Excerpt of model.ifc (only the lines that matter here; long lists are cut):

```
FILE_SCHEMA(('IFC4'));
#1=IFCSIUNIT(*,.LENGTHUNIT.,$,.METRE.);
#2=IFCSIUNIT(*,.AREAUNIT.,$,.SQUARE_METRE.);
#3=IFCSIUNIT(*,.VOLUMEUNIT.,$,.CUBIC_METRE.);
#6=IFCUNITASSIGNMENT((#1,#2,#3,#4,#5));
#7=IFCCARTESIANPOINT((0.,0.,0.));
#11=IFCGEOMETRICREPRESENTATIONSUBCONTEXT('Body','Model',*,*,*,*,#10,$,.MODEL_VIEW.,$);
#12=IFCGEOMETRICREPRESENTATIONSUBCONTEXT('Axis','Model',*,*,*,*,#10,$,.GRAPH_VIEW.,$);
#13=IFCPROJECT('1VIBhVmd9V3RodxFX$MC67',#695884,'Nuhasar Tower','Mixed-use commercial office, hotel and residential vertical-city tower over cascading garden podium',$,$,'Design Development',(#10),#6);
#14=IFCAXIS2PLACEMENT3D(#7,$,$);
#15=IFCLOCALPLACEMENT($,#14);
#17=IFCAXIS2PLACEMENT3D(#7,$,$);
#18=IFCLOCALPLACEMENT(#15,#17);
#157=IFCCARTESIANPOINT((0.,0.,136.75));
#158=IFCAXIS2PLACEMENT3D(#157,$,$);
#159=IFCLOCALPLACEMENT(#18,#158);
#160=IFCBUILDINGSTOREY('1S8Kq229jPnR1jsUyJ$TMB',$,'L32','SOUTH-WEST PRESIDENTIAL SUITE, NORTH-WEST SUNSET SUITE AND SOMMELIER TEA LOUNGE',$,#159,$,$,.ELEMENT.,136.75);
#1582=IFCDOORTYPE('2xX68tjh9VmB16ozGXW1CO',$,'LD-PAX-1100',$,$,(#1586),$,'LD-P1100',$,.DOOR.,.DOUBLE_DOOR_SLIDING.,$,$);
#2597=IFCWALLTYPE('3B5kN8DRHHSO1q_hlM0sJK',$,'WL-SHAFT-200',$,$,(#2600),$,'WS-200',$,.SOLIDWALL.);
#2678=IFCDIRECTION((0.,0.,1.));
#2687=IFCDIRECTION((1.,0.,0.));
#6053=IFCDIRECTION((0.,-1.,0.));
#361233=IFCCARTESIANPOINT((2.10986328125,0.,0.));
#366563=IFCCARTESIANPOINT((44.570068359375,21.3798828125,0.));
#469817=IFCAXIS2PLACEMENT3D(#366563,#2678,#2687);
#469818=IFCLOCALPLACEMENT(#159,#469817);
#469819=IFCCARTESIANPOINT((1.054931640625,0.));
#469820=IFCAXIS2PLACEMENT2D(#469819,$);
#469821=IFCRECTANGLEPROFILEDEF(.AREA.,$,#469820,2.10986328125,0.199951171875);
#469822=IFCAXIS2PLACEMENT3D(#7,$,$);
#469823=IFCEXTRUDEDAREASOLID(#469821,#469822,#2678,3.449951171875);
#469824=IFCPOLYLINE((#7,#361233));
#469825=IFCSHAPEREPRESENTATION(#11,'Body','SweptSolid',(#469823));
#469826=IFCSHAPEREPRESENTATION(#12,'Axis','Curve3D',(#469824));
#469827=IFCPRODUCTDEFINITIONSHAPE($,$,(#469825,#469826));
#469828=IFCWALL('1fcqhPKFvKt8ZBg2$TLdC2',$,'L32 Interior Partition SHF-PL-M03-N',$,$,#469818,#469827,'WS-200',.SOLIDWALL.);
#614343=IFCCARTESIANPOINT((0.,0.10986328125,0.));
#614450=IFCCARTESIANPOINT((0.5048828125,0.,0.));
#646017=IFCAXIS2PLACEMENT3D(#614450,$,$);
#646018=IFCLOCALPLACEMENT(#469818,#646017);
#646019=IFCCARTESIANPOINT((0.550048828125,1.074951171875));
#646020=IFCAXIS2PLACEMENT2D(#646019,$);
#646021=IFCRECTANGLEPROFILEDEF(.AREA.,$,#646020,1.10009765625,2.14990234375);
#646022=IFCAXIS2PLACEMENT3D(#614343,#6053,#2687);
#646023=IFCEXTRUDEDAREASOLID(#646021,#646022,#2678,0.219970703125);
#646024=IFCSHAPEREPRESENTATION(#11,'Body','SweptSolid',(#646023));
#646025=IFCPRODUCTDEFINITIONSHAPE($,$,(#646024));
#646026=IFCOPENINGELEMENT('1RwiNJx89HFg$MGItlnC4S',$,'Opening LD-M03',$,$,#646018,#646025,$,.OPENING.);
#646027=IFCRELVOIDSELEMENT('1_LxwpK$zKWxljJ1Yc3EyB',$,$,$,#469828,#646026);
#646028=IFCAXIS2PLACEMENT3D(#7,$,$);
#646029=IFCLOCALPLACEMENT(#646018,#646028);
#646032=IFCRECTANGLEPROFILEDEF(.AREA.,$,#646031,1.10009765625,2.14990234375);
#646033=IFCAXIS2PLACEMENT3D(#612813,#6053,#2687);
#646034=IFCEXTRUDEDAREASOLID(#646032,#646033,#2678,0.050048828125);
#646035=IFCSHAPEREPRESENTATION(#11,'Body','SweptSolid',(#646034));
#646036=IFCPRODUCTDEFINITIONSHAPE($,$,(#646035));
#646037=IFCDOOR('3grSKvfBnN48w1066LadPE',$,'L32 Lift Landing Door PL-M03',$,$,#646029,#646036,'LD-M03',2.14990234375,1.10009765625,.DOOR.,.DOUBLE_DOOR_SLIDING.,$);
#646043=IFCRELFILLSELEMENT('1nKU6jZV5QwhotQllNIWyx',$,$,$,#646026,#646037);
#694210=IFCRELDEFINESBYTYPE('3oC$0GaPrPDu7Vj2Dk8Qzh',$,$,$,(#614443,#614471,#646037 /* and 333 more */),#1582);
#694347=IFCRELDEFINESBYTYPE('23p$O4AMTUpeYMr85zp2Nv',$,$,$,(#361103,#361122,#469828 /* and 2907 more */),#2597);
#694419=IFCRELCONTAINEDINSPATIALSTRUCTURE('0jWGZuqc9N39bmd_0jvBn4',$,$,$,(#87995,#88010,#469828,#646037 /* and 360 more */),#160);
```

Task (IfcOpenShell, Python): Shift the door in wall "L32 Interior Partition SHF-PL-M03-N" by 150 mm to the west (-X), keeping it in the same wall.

```python
import ifcopenshell
import ifcopenshell.api.geometry
import ifcopenshell.util.placement
import ifcopenshell.util.unit

model = ifcopenshell.open("model.ifc")
unit_scale = ifcopenshell.util.unit.calculate_unit_scale(model)

door = model.by_id(646037)
opening = door.FillsVoids[0].RelatingOpeningElement
wall = opening.VoidsElements[0].RelatingBuildingElement

wall_matrix = ifcopenshell.util.placement.get_local_placement(wall.ObjectPlacement)
shift = wall_matrix[:3, 0] * -0.15 / unit_scale
before = ifcopenshell.util.placement.get_local_placement(door.ObjectPlacement)[:3, 3].copy()

# The door is placed relative to its opening, so it follows when the opening moves.
matrix = ifcopenshell.util.placement.get_local_placement(opening.ObjectPlacement)
matrix[:3, 3] += shift
ifcopenshell.api.geometry.edit_object_placement(
    model, product=opening, matrix=matrix, is_si=False, should_transform_children=True
)

after = ifcopenshell.util.placement.get_local_placement(door.ObjectPlacement)[:3, 3]
print("door moved by", (after - before).round(3) + 0.0)

model.write("model-out.ifc")
```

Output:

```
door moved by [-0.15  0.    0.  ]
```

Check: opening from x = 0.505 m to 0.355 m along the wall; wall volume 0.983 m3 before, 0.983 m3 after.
